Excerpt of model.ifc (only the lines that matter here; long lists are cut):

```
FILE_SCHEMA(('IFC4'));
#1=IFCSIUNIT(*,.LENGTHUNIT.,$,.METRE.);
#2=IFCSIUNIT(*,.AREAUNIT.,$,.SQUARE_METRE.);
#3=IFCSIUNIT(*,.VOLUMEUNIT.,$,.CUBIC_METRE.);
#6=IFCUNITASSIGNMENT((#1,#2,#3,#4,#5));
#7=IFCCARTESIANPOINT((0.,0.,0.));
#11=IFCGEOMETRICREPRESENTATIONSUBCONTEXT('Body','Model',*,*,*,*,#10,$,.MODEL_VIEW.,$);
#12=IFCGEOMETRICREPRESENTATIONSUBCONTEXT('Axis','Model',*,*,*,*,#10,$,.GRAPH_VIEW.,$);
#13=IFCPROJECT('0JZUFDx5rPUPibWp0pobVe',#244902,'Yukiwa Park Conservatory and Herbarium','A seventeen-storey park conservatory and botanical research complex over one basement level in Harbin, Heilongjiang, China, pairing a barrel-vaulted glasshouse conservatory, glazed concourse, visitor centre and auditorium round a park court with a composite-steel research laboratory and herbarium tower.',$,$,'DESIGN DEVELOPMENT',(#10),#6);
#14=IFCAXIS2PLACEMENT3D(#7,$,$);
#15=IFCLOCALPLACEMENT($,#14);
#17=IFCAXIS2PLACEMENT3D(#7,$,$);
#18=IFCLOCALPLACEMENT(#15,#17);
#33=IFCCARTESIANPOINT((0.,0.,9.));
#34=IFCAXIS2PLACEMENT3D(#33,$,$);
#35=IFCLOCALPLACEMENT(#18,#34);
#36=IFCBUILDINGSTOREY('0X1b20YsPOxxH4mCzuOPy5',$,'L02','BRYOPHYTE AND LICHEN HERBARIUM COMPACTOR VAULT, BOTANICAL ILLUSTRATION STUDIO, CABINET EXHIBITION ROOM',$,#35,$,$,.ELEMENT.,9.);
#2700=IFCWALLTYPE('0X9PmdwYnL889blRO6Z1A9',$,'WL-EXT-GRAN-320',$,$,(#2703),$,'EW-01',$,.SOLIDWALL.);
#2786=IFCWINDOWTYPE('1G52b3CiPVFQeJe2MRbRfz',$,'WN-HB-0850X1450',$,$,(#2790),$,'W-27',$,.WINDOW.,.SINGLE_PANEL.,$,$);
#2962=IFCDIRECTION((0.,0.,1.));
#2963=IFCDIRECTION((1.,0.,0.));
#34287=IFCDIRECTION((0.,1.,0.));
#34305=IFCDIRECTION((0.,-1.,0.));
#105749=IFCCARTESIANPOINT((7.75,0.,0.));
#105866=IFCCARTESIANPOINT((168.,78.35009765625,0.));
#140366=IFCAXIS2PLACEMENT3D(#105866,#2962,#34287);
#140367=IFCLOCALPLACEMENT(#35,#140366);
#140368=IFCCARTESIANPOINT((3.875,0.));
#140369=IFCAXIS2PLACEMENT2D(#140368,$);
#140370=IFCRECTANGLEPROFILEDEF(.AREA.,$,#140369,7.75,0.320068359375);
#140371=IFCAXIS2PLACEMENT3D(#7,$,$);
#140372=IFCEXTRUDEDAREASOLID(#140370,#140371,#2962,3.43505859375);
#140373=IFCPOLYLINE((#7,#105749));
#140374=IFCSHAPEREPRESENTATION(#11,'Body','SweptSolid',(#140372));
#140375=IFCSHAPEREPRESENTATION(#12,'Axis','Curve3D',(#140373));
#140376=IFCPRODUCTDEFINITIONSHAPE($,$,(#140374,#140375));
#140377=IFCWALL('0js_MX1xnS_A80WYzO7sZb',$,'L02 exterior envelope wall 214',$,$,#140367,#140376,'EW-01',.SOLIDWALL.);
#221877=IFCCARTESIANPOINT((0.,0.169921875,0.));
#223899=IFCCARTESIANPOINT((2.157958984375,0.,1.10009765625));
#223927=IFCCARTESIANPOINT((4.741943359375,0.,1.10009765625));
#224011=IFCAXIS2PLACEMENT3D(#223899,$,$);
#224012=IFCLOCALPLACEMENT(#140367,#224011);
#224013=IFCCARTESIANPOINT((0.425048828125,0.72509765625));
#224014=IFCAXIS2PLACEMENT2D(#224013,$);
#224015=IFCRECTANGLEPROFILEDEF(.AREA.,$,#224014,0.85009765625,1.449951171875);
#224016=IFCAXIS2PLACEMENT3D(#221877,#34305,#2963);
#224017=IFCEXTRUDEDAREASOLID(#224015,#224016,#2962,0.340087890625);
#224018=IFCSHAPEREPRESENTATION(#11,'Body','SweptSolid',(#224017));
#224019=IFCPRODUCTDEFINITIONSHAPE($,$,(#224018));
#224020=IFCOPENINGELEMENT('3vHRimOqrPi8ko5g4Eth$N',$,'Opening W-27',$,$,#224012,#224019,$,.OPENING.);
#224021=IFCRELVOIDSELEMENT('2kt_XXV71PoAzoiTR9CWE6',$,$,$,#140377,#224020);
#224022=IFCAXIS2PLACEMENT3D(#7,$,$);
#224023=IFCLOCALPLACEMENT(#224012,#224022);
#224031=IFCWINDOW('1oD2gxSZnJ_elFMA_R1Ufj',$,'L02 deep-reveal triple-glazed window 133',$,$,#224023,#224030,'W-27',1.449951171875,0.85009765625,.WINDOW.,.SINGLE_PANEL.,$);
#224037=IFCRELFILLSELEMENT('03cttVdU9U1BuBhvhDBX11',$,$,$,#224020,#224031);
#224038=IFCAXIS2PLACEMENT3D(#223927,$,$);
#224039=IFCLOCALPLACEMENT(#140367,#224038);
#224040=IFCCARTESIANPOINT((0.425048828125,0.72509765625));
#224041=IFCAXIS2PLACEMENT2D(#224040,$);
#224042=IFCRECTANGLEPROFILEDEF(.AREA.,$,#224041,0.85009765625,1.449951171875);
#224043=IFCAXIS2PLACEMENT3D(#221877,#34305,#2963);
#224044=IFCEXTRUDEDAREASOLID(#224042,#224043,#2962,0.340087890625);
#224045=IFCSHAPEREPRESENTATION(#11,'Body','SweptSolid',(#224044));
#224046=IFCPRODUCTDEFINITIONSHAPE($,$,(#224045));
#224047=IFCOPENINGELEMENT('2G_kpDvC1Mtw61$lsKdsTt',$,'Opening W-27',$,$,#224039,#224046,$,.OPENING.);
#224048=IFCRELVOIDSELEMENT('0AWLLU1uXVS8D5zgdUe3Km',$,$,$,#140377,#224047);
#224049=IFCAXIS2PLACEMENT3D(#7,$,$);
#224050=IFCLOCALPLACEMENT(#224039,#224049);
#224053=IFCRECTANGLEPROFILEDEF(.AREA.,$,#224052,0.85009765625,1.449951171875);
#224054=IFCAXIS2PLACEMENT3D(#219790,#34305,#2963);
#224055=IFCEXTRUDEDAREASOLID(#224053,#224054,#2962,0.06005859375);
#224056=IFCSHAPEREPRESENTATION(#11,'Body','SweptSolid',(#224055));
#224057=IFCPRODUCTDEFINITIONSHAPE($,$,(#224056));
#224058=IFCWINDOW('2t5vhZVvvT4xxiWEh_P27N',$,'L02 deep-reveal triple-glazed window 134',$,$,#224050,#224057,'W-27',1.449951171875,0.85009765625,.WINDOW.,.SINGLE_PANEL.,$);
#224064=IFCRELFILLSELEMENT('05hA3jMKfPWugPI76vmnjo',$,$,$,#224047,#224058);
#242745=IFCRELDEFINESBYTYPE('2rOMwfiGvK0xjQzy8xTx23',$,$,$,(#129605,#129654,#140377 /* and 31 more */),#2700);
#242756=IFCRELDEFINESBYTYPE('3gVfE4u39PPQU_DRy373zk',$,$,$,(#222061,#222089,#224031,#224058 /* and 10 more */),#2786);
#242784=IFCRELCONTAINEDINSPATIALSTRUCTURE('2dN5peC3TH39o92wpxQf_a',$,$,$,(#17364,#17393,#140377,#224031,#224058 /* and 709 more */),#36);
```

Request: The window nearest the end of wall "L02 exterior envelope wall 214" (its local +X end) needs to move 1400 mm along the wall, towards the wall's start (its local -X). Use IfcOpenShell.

```python
import ifcopenshell
import ifcopenshell.api.geometry
import ifcopenshell.util.placement

model = ifcopenshell.open("model.ifc")

window = model.by_id(224058)
opening = window.FillsVoids[0].RelatingOpeningElement
wall = opening.VoidsElements[0].RelatingBuildingElement

wall_matrix = ifcopenshell.util.placement.get_local_placement(wall.ObjectPlacement)
shift = wall_matrix[:3, 0] * -1.4
before = ifcopenshell.util.placement.get_local_placement(window.ObjectPlacement)[:3, 3].copy()

# The window is placed relative to its opening, so it follows when the opening moves.
matrix = ifcopenshell.util.placement.get_local_placement(opening.ObjectPlacement)
matrix[:3, 3] += shift
ifcopenshell.api.geometry.edit_object_placement(
    model, product=opening, matrix=matrix, is_si=False, should_transform_children=True
)

after = ifcopenshell.util.placement.get_local_placement(window.ObjectPlacement)[:3, 3]
print("window moved by", (after - before).round(3) + 0.0)

model.write("model-out.ifc")
```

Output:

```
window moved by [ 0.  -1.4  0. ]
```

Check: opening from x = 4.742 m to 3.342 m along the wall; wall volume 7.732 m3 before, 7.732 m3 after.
